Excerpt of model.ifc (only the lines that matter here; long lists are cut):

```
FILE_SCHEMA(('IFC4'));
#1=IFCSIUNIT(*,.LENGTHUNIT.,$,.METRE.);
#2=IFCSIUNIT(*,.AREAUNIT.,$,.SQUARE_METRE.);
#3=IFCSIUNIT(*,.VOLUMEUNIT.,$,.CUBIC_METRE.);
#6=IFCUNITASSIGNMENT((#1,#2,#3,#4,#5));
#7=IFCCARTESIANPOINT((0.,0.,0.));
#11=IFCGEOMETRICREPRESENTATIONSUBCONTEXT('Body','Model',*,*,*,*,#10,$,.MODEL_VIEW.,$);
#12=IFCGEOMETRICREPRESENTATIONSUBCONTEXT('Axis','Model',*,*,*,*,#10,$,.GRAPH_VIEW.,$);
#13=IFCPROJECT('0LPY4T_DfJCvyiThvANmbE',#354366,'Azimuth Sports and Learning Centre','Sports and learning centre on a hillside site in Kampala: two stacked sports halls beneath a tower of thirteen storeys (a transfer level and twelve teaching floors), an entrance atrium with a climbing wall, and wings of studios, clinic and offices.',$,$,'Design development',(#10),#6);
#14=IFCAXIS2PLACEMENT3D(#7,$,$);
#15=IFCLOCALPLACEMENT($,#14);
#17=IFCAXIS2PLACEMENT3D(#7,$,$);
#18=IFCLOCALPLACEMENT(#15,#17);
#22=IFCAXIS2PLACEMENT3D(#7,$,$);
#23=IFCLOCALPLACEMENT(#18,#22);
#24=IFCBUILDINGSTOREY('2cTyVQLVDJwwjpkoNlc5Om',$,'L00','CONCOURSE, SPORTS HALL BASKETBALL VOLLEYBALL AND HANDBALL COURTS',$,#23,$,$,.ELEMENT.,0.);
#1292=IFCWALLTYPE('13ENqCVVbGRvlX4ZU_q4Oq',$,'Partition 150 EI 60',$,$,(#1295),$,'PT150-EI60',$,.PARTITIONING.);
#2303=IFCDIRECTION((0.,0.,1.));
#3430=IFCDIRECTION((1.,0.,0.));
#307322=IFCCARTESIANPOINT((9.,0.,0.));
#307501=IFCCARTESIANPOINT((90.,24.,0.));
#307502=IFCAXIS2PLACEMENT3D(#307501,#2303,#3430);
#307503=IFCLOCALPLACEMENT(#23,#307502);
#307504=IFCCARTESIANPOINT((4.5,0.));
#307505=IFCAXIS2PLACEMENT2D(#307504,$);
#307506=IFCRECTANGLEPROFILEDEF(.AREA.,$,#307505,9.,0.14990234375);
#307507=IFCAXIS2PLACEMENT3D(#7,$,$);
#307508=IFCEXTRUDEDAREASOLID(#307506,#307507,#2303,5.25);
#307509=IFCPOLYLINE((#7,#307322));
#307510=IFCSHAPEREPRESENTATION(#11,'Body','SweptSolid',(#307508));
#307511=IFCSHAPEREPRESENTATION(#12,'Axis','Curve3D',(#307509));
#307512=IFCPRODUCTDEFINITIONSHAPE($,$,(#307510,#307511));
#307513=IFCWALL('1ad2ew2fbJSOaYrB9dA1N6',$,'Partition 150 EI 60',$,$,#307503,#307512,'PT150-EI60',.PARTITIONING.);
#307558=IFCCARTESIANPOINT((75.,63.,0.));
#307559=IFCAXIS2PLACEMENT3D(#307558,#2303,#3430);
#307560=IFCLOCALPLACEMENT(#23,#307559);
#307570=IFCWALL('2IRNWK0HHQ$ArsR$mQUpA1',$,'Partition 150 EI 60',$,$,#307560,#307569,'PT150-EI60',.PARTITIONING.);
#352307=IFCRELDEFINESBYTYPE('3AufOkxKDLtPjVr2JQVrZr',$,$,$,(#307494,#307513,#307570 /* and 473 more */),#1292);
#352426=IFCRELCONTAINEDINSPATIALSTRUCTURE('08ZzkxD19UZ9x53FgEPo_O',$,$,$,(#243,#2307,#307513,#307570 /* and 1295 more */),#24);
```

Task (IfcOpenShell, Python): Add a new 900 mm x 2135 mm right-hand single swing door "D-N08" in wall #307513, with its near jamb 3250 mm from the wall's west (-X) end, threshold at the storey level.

```python
import numpy as np
import ifcopenshell
import ifcopenshell.api.feature
import ifcopenshell.api.geometry
import ifcopenshell.api.root
import ifcopenshell.api.spatial
import ifcopenshell.geom
import ifcopenshell.util.element
import ifcopenshell.util.placement
import ifcopenshell.util.representation
import ifcopenshell.util.shape
import ifcopenshell.util.unit

model = ifcopenshell.open("model.ifc")
unit_scale = ifcopenshell.util.unit.calculate_unit_scale(model)
settings = ifcopenshell.geom.settings()


def volume(element):
    """Net volume in cubic metres, openings subtracted."""
    shape = ifcopenshell.geom.create_shape(settings, element)
    return ifcopenshell.util.shape.get_volume(shape.geometry)


wall = model.by_guid("1ad2ew2fbJSOaYrB9dA1N6")
storey = ifcopenshell.util.element.get_container(wall, ifc_class="IfcBuildingStorey")
context = ifcopenshell.util.representation.get_context(model, "Model", "Body", "MODEL_VIEW")
before = volume(wall)

width, height, from_end, sill = 0.9, 2.135, 3.25, 0.0  # metres

# The wall runs along its own X axis, and the end named is its -X end.
wall_shape = ifcopenshell.geom.create_shape(settings, wall)
x, y, z = ifcopenshell.util.shape.get_vertices(wall_shape.geometry).T
start = x.min() + from_end
face, thickness = float(y.min()), float(y.max() - y.min())
wall_matrix = ifcopenshell.util.placement.get_local_placement(wall.ObjectPlacement)
level = ifcopenshell.util.placement.get_local_placement(storey.ObjectPlacement)[2, 3]


def in_wall(x, y):
    """Placement at x, y metres in the wall's axes, at sill height."""
    matrix = wall_matrix.copy()
    matrix[:, 3] = wall_matrix @ np.array([x / unit_scale, y / unit_scale, 0.0, 1.0])
    matrix[2, 3] = level + sill / unit_scale
    return matrix


# Opening: a box that overshoots both wall faces by 50 mm.
opening = ifcopenshell.api.root.create_entity(model, ifc_class="IfcOpeningElement", predefined_type="OPENING")
box = ifcopenshell.api.geometry.add_wall_representation(
    model, context=context, length=width, height=height, thickness=thickness + 0.1
)
ifcopenshell.api.geometry.assign_representation(model, product=opening, representation=box)
ifcopenshell.api.geometry.edit_object_placement(model, product=opening, matrix=in_wall(start, face - 0.05), is_si=False)
ifcopenshell.api.feature.add_feature(model, feature=opening, element=wall)

door = ifcopenshell.api.root.create_entity(model, ifc_class="IfcDoor", name="D-N08", predefined_type="DOOR")
door.OverallWidth, door.OverallHeight = width / unit_scale, height / unit_scale
door.OperationType = "SINGLE_SWING_RIGHT"
body = ifcopenshell.api.geometry.add_door_representation(
    model,
    context=context,
    overall_width=door.OverallWidth,
    overall_height=door.OverallHeight,
    operation_type="SINGLE_SWING_RIGHT",
    lining_properties={"LiningDepth": thickness / unit_scale, "ThresholdDepth": thickness / unit_scale},
)
ifcopenshell.api.geometry.assign_representation(model, product=door, representation=body)
ifcopenshell.api.spatial.assign_container(model, products=[door], relating_structure=storey)
ifcopenshell.api.feature.add_filling(model, opening=opening, element=door)

# The lining spans the wall, so the door starts at the wall face.
ifcopenshell.api.geometry.edit_object_placement(model, product=door, matrix=in_wall(start, face), is_si=False)

after = volume(wall)

print(f"wall volume {before:.3f} -> {after:.3f} m3")

model.write("model_v2.ifc")
```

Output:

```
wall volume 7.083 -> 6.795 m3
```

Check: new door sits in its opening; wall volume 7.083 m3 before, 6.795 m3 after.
